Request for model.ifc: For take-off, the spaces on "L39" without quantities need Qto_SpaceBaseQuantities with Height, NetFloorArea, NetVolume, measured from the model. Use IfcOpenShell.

First a look at what the model holds.

```python
import ifcopenshell
import ifcopenshell.util.element
import ifcopenshell.util.unit

model = ifcopenshell.open("model.ifc")
print(model.schema)
for unit_type in ("LENGTHUNIT", "AREAUNIT", "VOLUMEUNIT"):
    print(unit_type, ifcopenshell.util.unit.calculate_unit_scale(model, unit_type))
storey = next(s for s in model.by_type("IfcBuildingStorey") if s.Name == "L39")
spaces = [e for e in ifcopenshell.util.element.get_decomposition(storey) if e.is_a("IfcSpace")]
for e in sorted(spaces, key=lambda e: e.id()):
    print(e.id(), e.is_a(), e.Name, list(ifcopenshell.util.element.get_psets(e, qtos_only=True)), sep=" | ")
```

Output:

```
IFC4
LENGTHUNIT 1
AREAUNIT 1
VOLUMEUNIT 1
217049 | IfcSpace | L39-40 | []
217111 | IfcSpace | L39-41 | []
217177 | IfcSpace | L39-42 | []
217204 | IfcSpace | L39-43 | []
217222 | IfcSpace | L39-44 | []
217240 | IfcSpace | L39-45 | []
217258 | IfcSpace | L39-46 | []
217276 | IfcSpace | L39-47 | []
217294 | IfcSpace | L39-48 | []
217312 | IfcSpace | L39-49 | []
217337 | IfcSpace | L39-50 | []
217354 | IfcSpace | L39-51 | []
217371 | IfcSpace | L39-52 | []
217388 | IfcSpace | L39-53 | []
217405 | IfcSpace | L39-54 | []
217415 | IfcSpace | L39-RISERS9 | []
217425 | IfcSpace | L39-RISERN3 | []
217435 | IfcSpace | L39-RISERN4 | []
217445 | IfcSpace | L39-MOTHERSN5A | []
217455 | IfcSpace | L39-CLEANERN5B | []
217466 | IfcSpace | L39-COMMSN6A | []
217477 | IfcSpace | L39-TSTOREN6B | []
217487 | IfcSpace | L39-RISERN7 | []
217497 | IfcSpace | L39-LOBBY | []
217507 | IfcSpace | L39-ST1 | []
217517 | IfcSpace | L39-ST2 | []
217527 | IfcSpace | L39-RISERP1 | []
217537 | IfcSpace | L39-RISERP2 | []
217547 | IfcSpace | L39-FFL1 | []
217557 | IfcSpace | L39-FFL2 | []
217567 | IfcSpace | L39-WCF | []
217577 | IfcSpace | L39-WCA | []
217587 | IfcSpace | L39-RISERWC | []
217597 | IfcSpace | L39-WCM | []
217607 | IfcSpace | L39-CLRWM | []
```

```python
import ifcopenshell
import ifcopenshell.api.pset
import ifcopenshell.geom
import ifcopenshell.util.element
import ifcopenshell.util.shape
import ifcopenshell.util.unit

model = ifcopenshell.open("model.ifc")
unit_scale = ifcopenshell.util.unit.calculate_unit_scale(model)
area_scale = ifcopenshell.util.unit.calculate_unit_scale(model, "AREAUNIT")
volume_scale = ifcopenshell.util.unit.calculate_unit_scale(model, "VOLUMEUNIT")
settings = ifcopenshell.geom.settings()

storey = next(s for s in model.by_type("IfcBuildingStorey") if s.Name == "L39")
spaces = [e for e in ifcopenshell.util.element.get_decomposition(storey) if e.is_a("IfcSpace")]

for e in sorted(spaces, key=lambda e: e.id()):
    if ifcopenshell.util.element.get_psets(e, qtos_only=True, should_inherit=False):
        continue
    # Geometry comes back in metres, in the element's own axes.
    shape = ifcopenshell.geom.create_shape(settings, e)
    values = {
        "Height": ifcopenshell.util.shape.get_z(shape.geometry) / unit_scale,
        "NetFloorArea": ifcopenshell.util.shape.get_footprint_area(shape.geometry) / area_scale,
        "NetVolume": ifcopenshell.util.shape.get_volume(shape.geometry) / volume_scale,
    }
    qto = ifcopenshell.api.pset.add_qto(model, product=e, name="Qto_SpaceBaseQuantities")
    ifcopenshell.api.pset.edit_qto(model, qto=qto, properties=values)
    print(e.id(), {k: round(v, 3) for k, v in values.items()})

model.write("model_rev.ifc")
```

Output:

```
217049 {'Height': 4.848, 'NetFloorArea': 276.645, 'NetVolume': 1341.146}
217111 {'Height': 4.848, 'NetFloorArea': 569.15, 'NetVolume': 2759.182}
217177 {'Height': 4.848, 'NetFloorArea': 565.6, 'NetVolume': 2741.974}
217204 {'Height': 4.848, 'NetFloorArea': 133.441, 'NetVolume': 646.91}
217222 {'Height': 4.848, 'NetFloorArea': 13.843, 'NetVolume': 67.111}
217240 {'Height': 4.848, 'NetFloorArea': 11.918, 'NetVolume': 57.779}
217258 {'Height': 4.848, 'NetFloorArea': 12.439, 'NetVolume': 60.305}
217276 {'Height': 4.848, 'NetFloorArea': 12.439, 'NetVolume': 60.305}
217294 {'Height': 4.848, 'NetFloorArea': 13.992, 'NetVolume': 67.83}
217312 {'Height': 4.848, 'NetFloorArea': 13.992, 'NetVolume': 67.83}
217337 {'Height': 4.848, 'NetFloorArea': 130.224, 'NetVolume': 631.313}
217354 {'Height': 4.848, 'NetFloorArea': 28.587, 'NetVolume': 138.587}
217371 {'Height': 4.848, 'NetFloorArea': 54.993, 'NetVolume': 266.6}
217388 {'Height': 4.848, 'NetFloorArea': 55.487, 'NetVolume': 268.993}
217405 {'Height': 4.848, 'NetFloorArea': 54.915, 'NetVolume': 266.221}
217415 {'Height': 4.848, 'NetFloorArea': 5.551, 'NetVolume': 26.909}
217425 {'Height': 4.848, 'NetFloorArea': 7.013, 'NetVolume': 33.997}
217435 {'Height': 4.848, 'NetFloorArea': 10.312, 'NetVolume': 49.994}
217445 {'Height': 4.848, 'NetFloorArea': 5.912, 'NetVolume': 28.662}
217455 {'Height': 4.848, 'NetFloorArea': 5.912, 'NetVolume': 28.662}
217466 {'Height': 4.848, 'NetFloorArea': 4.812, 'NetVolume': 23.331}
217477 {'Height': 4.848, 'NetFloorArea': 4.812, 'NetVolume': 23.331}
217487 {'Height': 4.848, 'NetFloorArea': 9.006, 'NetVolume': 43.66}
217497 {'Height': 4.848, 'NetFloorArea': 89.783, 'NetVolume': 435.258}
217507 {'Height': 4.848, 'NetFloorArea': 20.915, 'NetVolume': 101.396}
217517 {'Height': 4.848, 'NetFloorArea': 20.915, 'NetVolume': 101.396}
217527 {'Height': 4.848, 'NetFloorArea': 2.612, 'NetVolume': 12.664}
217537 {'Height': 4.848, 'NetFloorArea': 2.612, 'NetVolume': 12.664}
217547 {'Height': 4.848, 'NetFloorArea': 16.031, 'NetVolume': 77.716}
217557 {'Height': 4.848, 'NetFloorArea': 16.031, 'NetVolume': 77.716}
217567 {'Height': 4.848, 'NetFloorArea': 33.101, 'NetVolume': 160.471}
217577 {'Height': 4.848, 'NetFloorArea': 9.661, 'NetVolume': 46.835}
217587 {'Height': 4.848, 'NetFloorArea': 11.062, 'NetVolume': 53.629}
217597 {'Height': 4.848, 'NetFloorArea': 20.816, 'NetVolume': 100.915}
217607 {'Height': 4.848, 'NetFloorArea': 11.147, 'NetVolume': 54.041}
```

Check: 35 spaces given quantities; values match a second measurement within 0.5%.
